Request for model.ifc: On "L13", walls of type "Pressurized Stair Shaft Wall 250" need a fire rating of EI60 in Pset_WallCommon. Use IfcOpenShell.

First a look at what the model holds.

```python
import ifcopenshell
import ifcopenshell.util.element

model = ifcopenshell.open("model.ifc")
print(model.schema)
storey = next(s for s in model.by_type("IfcBuildingStorey") if s.Name == "L13")
walls = [e for e in ifcopenshell.util.element.get_decomposition(storey) if e.is_a("IfcWall")]
seen = {}
for e in walls:
    element_type = ifcopenshell.util.element.get_type(e)
    key = (element_type.Name if element_type != e and element_type else None, ifcopenshell.util.element.get_pset(e, "Pset_WallCommon", "FireRating"))
    seen[key] = seen.get(key, 0) + 1
for (name, value), count in sorted(seen.items(), key=str):
    print(count, "x", name, "|", value)
```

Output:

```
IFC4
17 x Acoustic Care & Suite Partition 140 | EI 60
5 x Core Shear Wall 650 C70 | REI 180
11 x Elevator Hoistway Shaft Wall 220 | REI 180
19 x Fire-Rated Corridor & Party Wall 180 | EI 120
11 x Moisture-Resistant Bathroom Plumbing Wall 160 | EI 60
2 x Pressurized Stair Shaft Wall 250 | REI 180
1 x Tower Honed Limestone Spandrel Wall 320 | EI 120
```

```python
import ifcopenshell
import ifcopenshell.api.pset
import ifcopenshell.util.element

model = ifcopenshell.open("model.ifc")

storey = next(s for s in model.by_type("IfcBuildingStorey") if s.Name == "L13")
walls = [e for e in ifcopenshell.util.element.get_decomposition(storey) if e.is_a("IfcWall")]

count = 0
for e in walls:
    element_type = ifcopenshell.util.element.get_type(e)
    if element_type in (None, e) or element_type.Name != "Pressurized Stair Shaft Wall 250":
        continue
    found = ifcopenshell.util.element.get_pset(e, "Pset_WallCommon", should_inherit=False)
    if found:
        pset = model.by_id(found["id"])
        if len(ifcopenshell.util.element.get_elements_by_pset(pset)) > 1:
            pset = ifcopenshell.api.pset.unshare_pset(model, products=[e], pset=pset)[0]
    else:
        pset = ifcopenshell.api.pset.add_pset(model, product=e, name="Pset_WallCommon")
    ifcopenshell.api.pset.edit_pset(model, pset=pset, properties={"FireRating": "EI60"})
    count += 1

print(count, "walls updated")

model.write("model-out.ifc")
```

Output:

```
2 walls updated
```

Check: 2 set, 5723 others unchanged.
